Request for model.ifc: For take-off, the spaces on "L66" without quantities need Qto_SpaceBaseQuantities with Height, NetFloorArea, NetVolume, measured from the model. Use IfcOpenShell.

First a look at what the model holds.

```python
import ifcopenshell
import ifcopenshell.util.element
import ifcopenshell.util.unit

model = ifcopenshell.open("model.ifc")
print(model.schema)
for unit_type in ("LENGTHUNIT", "AREAUNIT", "VOLUMEUNIT"):
    print(unit_type, ifcopenshell.util.unit.calculate_unit_scale(model, unit_type))
storey = next(s for s in model.by_type("IfcBuildingStorey") if s.Name == "L66")
spaces = [e for e in ifcopenshell.util.element.get_decomposition(storey) if e.is_a("IfcSpace")]
for e in sorted(spaces, key=lambda e: e.id()):
    print(e.id(), e.is_a(), e.Name, list(ifcopenshell.util.element.get_psets(e, qtos_only=True)), sep=" | ")
```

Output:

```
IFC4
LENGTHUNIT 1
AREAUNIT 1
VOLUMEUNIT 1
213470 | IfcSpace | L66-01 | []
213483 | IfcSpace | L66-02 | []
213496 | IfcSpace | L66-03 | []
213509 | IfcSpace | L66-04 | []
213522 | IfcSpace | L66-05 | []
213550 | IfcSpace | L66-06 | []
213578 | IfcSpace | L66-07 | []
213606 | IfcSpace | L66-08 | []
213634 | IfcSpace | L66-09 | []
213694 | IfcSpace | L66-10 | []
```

```python
import ifcopenshell
import ifcopenshell.api.pset
import ifcopenshell.geom
import ifcopenshell.util.element
import ifcopenshell.util.shape
import ifcopenshell.util.unit

model = ifcopenshell.open("model.ifc")
unit_scale = ifcopenshell.util.unit.calculate_unit_scale(model)
area_scale = ifcopenshell.util.unit.calculate_unit_scale(model, "AREAUNIT")
volume_scale = ifcopenshell.util.unit.calculate_unit_scale(model, "VOLUMEUNIT")
settings = ifcopenshell.geom.settings()

storey = next(s for s in model.by_type("IfcBuildingStorey") if s.Name == "L66")
spaces = [e for e in ifcopenshell.util.element.get_decomposition(storey) if e.is_a("IfcSpace")]

for e in sorted(spaces, key=lambda e: e.id()):
    if ifcopenshell.util.element.get_psets(e, qtos_only=True, should_inherit=False):
        continue
    # Geometry comes back in metres, in the element's own axes.
    shape = ifcopenshell.geom.create_shape(settings, e)
    values = {
        "Height": ifcopenshell.util.shape.get_z(shape.geometry) / unit_scale,
        "NetFloorArea": ifcopenshell.util.shape.get_footprint_area(shape.geometry) / area_scale,
        "NetVolume": ifcopenshell.util.shape.get_volume(shape.geometry) / volume_scale,
    }
    qto = ifcopenshell.api.pset.add_qto(model, product=e, name="Qto_SpaceBaseQuantities")
    ifcopenshell.api.pset.edit_qto(model, qto=qto, properties=values)
    print(e.id(), {k: round(v, 3) for k, v in values.items()})

model.write("model_updated.ifc")
```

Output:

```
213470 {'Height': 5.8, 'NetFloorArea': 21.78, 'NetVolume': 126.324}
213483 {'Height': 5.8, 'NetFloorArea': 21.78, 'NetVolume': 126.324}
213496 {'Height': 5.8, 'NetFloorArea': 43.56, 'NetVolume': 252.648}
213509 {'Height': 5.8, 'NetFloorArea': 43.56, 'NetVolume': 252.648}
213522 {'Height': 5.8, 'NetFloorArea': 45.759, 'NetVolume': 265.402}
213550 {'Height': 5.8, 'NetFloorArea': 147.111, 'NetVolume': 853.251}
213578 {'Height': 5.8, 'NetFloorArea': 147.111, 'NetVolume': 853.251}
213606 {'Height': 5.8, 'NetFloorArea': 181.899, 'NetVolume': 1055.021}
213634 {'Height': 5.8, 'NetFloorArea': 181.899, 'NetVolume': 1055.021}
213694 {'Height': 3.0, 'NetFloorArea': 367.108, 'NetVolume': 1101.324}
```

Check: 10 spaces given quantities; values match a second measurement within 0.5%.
